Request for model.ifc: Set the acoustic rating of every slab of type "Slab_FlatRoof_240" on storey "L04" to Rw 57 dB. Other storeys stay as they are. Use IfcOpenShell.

First a look at what the model holds.

```python
import ifcopenshell
import ifcopenshell.util.element

model = ifcopenshell.open("model.ifc")
print(model.schema)
storey = next(s for s in model.by_type("IfcBuildingStorey") if s.Name == "L04")
slabs = [e for e in ifcopenshell.util.element.get_decomposition(storey) if e.is_a("IfcSlab")]
seen = {}
for e in slabs:
    element_type = ifcopenshell.util.element.get_type(e)
    key = (element_type.Name if element_type != e and element_type else None, ifcopenshell.util.element.get_pset(e, "Pset_SlabCommon", "AcousticRating"))
    seen[key] = seen.get(key, 0) + 1
for (name, value), count in sorted(seen.items(), key=str):
    print(count, "x", name, "|", value)
```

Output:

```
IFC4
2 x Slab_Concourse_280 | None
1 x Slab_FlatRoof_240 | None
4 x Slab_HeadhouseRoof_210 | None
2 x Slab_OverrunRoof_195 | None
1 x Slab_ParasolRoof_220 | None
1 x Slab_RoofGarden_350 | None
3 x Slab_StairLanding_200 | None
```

```python
import ifcopenshell
import ifcopenshell.api.pset
import ifcopenshell.util.element

model = ifcopenshell.open("model.ifc")

storey = next(s for s in model.by_type("IfcBuildingStorey") if s.Name == "L04")
slabs = [e for e in ifcopenshell.util.element.get_decomposition(storey) if e.is_a("IfcSlab")]

count = 0
for e in slabs:
    element_type = ifcopenshell.util.element.get_type(e)
    if element_type in (None, e) or element_type.Name != "Slab_FlatRoof_240":
        continue
    # add_pset returns the element's existing set when there is one.
    pset = ifcopenshell.api.pset.add_pset(model, product=e, name="Pset_SlabCommon")
    ifcopenshell.api.pset.edit_pset(model, pset=pset, properties={"AcousticRating": "Rw 57 dB"})
    count += 1

print(count, "slabs updated")

model.write("model_updated.ifc")
```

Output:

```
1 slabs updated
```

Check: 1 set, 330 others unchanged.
